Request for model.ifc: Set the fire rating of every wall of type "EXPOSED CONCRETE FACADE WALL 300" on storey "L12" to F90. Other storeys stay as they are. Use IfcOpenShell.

First a look at what the model holds.

```python
import ifcopenshell
import ifcopenshell.util.element

model = ifcopenshell.open("model.ifc")
print(model.schema)
storey = next(s for s in model.by_type("IfcBuildingStorey") if s.Name == "L12")
walls = [e for e in ifcopenshell.util.element.get_decomposition(storey) if e.is_a("IfcWall")]
seen = {}
for e in walls:
    element_type = ifcopenshell.util.element.get_type(e)
    key = (element_type.Name if element_type != e and element_type else None, ifcopenshell.util.element.get_pset(e, "Pset_WallCommon", "FireRating"))
    seen[key] = seen.get(key, 0) + 1
for (name, value), count in sorted(seen.items(), key=str):
    print(count, "x", name, "|", value)
```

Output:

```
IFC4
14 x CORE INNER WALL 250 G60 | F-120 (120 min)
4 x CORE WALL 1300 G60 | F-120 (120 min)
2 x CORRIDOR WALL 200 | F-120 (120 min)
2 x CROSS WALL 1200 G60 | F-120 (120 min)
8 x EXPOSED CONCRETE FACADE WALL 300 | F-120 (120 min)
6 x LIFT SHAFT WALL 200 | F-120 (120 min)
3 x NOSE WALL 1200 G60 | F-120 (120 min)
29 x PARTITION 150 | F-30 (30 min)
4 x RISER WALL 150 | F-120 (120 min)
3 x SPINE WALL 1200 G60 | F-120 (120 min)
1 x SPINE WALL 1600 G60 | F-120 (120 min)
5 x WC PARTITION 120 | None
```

```python
import ifcopenshell
import ifcopenshell.api.pset
import ifcopenshell.util.element

model = ifcopenshell.open("model.ifc")

storey = next(s for s in model.by_type("IfcBuildingStorey") if s.Name == "L12")
walls = [e for e in ifcopenshell.util.element.get_decomposition(storey) if e.is_a("IfcWall")]

count = 0
for e in walls:
    element_type = ifcopenshell.util.element.get_type(e)
    if element_type in (None, e) or element_type.Name != "EXPOSED CONCRETE FACADE WALL 300":
        continue
    found = ifcopenshell.util.element.get_pset(e, "Pset_WallCommon", should_inherit=False)
    if found:
        pset = model.by_id(found["id"])
        if len(ifcopenshell.util.element.get_elements_by_pset(pset)) > 1:
            pset = ifcopenshell.api.pset.unshare_pset(model, products=[e], pset=pset)[0]
    else:
        pset = ifcopenshell.api.pset.add_pset(model, product=e, name="Pset_WallCommon")
    ifcopenshell.api.pset.edit_pset(model, pset=pset, properties={"FireRating": "F90"})
    count += 1

print(count, "walls updated")

model.write("model_rev.ifc")
```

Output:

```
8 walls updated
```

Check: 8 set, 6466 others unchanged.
